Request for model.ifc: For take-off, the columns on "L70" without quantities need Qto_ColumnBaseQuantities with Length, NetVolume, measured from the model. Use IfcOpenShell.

First a look at what the model holds.

```python
import ifcopenshell
import ifcopenshell.util.element
import ifcopenshell.util.unit

model = ifcopenshell.open("model.ifc")
print(model.schema)
for unit_type in ("LENGTHUNIT", "AREAUNIT", "VOLUMEUNIT"):
    print(unit_type, ifcopenshell.util.unit.calculate_unit_scale(model, unit_type))
storey = next(s for s in model.by_type("IfcBuildingStorey") if s.Name == "L70")
columns = [e for e in ifcopenshell.util.element.get_decomposition(storey) if e.is_a("IfcColumn")]
for e in sorted(columns, key=lambda e: e.id()):
    print(e.id(), e.is_a(), e.Name, list(ifcopenshell.util.element.get_psets(e, qtos_only=True)), sep=" | ")
```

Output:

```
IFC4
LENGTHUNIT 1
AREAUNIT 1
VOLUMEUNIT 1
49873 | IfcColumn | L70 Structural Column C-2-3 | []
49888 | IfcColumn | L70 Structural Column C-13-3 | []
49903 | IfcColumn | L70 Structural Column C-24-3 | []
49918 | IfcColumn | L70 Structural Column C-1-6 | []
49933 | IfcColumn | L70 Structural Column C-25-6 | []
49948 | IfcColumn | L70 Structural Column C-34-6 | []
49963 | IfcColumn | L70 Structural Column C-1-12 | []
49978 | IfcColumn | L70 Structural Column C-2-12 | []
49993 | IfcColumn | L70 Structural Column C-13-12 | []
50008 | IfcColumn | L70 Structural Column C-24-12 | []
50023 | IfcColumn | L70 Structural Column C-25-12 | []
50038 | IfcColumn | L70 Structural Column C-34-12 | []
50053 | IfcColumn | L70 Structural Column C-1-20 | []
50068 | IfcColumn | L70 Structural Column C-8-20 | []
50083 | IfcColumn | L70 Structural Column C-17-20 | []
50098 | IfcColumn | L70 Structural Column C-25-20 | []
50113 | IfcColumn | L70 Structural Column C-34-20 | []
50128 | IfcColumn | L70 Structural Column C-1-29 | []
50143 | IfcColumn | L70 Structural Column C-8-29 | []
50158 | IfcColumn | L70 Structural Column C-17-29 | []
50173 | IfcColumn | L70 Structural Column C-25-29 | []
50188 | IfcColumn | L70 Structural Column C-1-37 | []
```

```python
import ifcopenshell
import ifcopenshell.api.pset
import ifcopenshell.geom
import ifcopenshell.util.element
import ifcopenshell.util.shape
import ifcopenshell.util.unit

model = ifcopenshell.open("model.ifc")
unit_scale = ifcopenshell.util.unit.calculate_unit_scale(model)
volume_scale = ifcopenshell.util.unit.calculate_unit_scale(model, "VOLUMEUNIT")
settings = ifcopenshell.geom.settings()

storey = next(s for s in model.by_type("IfcBuildingStorey") if s.Name == "L70")
columns = [e for e in ifcopenshell.util.element.get_decomposition(storey) if e.is_a("IfcColumn")]

for e in sorted(columns, key=lambda e: e.id()):
    if ifcopenshell.util.element.get_psets(e, qtos_only=True, should_inherit=False):
        continue
    # Geometry comes back in metres, in the element's own axes.
    shape = ifcopenshell.geom.create_shape(settings, e)
    values = {
        "Length": ifcopenshell.util.shape.get_z(shape.geometry) / unit_scale,
        "NetVolume": ifcopenshell.util.shape.get_volume(shape.geometry) / volume_scale,
    }
    qto = ifcopenshell.api.pset.add_qto(model, product=e, name="Qto_ColumnBaseQuantities")
    ifcopenshell.api.pset.edit_qto(model, qto=qto, properties=values)
    print(e.id(), {k: round(v, 3) for k, v in values.items()})

model.write("model_updated.ifc")
```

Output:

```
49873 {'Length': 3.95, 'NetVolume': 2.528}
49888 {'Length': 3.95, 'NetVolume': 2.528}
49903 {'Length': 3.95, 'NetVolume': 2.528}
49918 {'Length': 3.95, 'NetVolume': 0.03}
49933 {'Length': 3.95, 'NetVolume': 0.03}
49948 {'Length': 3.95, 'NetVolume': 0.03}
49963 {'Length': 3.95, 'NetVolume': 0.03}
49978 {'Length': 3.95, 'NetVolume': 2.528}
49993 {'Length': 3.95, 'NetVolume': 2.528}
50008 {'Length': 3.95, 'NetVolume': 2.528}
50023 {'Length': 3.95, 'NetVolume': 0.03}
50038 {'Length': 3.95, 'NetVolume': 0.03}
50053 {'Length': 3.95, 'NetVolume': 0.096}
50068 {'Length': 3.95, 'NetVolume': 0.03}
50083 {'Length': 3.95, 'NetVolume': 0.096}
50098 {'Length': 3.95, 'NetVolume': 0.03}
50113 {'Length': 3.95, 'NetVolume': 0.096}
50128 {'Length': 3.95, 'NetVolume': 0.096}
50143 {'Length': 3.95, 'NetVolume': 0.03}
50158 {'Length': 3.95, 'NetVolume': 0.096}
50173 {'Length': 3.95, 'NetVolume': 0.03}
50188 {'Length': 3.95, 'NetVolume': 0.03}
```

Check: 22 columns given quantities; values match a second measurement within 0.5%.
